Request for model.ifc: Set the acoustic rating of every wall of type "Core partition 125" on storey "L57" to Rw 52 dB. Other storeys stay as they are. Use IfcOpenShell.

First a look at what the model holds.

```python
import ifcopenshell
import ifcopenshell.util.element

model = ifcopenshell.open("model.ifc")
print(model.schema)
storey = next(s for s in model.by_type("IfcBuildingStorey") if s.Name == "L57")
walls = [e for e in ifcopenshell.util.element.get_decomposition(storey) if e.is_a("IfcWall")]
seen = {}
for e in walls:
    element_type = ifcopenshell.util.element.get_type(e)
    key = (element_type.Name if element_type != e and element_type else None, ifcopenshell.util.element.get_pset(e, "Pset_WallCommon", "AcousticRating"))
    seen[key] = seen.get(key, 0) + 1
for (name, value), count in sorted(seen.items(), key=str):
    print(count, "x", name, "|", value)
```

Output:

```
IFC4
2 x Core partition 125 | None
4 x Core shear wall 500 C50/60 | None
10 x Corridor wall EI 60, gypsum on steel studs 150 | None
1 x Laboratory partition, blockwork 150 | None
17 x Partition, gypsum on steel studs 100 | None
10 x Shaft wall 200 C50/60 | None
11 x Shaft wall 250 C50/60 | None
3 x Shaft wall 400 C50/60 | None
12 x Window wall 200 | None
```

```python
import ifcopenshell
import ifcopenshell.api.pset
import ifcopenshell.util.element

model = ifcopenshell.open("model.ifc")

storey = next(s for s in model.by_type("IfcBuildingStorey") if s.Name == "L57")
walls = [e for e in ifcopenshell.util.element.get_decomposition(storey) if e.is_a("IfcWall")]

count = 0
for e in walls:
    element_type = ifcopenshell.util.element.get_type(e)
    if element_type in (None, e) or element_type.Name != "Core partition 125":
        continue
    found = ifcopenshell.util.element.get_pset(e, "Pset_WallCommon", should_inherit=False)
    if found:
        pset = model.by_id(found["id"])
        if len(ifcopenshell.util.element.get_elements_by_pset(pset)) > 1:
            pset = ifcopenshell.api.pset.unshare_pset(model, products=[e], pset=pset)[0]
    else:
        pset = ifcopenshell.api.pset.add_pset(model, product=e, name="Pset_WallCommon")
    ifcopenshell.api.pset.edit_pset(model, pset=pset, properties={"AcousticRating": "Rw 52 dB"})
    count += 1

print(count, "walls updated")

model.write("model_rev.ifc")
```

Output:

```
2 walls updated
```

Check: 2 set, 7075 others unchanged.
